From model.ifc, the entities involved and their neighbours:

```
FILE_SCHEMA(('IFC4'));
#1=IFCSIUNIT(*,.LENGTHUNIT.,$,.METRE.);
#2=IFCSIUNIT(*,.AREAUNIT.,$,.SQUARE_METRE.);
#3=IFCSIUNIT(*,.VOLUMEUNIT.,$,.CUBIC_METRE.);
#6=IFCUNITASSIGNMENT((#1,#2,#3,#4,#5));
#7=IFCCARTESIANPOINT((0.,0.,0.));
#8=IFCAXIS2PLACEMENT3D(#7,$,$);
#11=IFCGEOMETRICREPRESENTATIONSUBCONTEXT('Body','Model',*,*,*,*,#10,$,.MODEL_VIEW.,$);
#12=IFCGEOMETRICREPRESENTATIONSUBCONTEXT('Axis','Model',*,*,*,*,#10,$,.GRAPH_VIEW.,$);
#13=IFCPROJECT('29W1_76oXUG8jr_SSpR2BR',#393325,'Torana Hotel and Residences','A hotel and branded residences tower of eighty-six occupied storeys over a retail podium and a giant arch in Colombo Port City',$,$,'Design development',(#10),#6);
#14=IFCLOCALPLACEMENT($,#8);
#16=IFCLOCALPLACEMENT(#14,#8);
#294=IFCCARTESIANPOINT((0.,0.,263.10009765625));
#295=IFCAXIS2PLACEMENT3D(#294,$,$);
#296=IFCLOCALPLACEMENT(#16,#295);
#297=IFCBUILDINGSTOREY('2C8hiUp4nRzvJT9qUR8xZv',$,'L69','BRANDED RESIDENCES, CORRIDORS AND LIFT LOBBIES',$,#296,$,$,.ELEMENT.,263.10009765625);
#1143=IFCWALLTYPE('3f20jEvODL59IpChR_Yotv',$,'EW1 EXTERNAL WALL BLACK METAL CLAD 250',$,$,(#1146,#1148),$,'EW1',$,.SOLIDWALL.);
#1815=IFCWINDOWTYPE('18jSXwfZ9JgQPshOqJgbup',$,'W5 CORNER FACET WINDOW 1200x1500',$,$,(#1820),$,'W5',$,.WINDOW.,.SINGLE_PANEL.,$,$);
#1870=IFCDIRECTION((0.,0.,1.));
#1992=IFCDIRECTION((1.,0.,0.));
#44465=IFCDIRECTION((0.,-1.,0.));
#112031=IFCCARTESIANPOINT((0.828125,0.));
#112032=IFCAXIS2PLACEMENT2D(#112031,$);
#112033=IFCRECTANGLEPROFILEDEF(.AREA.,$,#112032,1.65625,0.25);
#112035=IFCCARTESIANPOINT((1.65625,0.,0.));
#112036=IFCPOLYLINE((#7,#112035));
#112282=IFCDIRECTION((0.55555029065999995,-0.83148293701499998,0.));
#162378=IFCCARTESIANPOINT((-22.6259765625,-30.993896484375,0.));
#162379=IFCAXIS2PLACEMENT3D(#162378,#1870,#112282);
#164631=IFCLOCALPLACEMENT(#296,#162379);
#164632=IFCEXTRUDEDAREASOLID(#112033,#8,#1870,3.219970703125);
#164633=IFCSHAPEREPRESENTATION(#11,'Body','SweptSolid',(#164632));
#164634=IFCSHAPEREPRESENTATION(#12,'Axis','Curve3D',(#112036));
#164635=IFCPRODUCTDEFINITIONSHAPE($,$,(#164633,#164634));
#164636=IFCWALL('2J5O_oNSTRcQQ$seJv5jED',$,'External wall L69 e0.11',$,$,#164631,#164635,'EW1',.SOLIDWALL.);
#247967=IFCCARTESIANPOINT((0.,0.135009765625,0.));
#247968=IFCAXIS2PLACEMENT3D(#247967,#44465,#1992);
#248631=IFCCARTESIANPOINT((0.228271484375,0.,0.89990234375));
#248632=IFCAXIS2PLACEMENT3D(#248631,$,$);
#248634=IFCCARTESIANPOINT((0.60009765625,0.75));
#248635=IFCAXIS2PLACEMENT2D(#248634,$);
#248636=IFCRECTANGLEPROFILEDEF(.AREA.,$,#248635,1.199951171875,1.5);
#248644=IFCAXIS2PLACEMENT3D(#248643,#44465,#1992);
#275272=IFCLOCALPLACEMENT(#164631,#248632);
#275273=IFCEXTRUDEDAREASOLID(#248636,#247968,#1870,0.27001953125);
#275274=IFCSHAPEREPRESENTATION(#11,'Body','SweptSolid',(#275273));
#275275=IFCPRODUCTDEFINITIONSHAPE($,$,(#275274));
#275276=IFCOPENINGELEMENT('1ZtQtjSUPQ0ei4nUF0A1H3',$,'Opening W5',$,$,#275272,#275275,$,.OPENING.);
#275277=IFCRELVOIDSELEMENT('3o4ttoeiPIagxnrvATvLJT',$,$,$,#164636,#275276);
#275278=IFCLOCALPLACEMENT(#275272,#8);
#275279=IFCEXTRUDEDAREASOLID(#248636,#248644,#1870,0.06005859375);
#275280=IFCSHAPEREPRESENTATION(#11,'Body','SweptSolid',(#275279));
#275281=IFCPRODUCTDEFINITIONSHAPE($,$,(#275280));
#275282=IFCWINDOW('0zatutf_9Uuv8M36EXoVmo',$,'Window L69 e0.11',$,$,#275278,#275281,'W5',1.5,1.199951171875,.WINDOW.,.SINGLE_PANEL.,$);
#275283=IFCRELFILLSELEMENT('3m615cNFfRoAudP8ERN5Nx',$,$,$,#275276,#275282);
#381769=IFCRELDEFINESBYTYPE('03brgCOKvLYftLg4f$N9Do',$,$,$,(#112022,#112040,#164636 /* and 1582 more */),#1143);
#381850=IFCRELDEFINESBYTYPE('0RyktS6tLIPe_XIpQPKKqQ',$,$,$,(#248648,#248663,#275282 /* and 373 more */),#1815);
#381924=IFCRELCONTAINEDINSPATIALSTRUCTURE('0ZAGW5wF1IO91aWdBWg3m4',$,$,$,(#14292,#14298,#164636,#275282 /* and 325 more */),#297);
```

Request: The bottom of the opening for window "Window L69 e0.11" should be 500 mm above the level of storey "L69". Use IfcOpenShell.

```python
import numpy as np
import ifcopenshell
import ifcopenshell.api.geometry
import ifcopenshell.geom
import ifcopenshell.util.element
import ifcopenshell.util.placement
import ifcopenshell.util.shape
import ifcopenshell.util.unit

model = ifcopenshell.open("model.ifc")
unit_scale = ifcopenshell.util.unit.calculate_unit_scale(model)

window = model.by_guid("0zatutf_9Uuv8M36EXoVmo")
opening = window.FillsVoids[0].RelatingOpeningElement
storey = ifcopenshell.util.element.get_container(window, ifc_class="IfcBuildingStorey")
level = ifcopenshell.util.placement.get_local_placement(storey.ObjectPlacement)[2, 3]

# The opening's origin need not be at the sill, so measure its lowest point.
shape = ifcopenshell.geom.create_shape(ifcopenshell.geom.settings(), opening)
bottom = ifcopenshell.util.shape.get_shape_bottom_elevation(shape, shape.geometry) / unit_scale
dz = level + 0.5 / unit_scale - bottom

shift = np.array([0.0, 0.0, dz])
# The window is placed relative to its opening, so it follows when the opening moves.
matrix = ifcopenshell.util.placement.get_local_placement(opening.ObjectPlacement)
matrix[:3, 3] += shift
ifcopenshell.api.geometry.edit_object_placement(
    model, product=opening, matrix=matrix, is_si=False, should_transform_children=True
)

print(f"moved by {dz * unit_scale:+.3f} m")

model.write("model_edited.ifc")
```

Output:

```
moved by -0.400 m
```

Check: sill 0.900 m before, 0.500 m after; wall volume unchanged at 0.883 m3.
